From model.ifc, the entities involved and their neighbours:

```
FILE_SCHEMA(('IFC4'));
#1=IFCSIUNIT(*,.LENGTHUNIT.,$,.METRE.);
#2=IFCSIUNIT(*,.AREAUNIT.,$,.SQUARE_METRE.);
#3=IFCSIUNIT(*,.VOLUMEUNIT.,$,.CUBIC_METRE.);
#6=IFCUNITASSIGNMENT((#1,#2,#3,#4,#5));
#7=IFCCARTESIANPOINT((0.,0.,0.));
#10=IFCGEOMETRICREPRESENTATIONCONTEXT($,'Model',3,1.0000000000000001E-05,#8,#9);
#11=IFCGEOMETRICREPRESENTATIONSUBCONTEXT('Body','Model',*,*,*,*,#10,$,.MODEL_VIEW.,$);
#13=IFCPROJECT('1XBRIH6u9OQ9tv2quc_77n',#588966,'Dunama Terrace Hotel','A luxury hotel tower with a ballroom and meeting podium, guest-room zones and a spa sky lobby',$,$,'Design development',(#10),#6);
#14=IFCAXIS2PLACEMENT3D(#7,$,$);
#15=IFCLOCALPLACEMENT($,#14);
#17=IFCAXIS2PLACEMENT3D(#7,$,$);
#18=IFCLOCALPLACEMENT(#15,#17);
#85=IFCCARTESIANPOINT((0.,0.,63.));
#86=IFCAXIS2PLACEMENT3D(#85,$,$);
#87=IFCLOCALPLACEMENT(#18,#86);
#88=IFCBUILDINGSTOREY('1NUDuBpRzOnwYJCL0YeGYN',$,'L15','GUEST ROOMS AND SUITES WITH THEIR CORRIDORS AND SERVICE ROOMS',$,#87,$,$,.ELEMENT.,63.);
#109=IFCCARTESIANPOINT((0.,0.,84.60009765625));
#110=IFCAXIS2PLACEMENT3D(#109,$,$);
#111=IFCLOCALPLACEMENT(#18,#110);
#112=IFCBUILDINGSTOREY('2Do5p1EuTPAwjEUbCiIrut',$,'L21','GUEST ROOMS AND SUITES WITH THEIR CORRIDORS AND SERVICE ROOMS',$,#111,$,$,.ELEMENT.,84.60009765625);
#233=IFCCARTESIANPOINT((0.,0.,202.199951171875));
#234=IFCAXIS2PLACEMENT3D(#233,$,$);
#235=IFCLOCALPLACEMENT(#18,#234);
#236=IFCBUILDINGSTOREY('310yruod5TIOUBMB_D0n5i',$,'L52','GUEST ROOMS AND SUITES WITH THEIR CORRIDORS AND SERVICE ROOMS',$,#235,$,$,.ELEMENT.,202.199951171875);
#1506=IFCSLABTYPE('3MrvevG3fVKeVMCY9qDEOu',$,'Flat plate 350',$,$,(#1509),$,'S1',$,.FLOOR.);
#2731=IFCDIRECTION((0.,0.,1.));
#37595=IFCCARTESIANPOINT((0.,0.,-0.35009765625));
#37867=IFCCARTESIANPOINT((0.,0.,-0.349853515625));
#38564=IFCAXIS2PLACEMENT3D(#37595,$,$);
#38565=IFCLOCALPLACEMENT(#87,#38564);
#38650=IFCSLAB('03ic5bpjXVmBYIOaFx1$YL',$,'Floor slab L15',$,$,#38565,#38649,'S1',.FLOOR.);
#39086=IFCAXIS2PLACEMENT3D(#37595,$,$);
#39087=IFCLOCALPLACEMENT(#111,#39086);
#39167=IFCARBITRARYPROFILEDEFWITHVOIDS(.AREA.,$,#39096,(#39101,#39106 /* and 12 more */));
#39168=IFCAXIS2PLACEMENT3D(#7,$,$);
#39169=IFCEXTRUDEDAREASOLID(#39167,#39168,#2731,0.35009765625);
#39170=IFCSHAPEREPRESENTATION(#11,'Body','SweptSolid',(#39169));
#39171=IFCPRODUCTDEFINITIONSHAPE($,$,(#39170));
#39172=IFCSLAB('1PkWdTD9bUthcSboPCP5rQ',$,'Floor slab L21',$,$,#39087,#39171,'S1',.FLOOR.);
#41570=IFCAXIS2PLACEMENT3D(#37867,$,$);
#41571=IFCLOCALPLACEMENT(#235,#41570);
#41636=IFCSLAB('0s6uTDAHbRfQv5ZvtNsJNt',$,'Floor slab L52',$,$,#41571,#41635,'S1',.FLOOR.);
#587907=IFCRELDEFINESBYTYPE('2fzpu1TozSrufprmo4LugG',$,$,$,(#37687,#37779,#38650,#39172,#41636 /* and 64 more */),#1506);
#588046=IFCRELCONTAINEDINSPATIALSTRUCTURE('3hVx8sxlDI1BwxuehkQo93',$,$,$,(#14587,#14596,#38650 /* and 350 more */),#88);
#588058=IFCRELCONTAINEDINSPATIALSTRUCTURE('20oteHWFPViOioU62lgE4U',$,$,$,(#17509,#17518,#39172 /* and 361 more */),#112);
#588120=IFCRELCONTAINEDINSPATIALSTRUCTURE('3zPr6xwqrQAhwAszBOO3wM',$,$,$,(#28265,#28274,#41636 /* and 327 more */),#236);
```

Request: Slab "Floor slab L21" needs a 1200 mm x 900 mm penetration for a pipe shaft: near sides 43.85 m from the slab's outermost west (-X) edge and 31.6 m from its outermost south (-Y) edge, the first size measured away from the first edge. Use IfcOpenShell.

```python
import numpy as np
import ifcopenshell
import ifcopenshell.api.feature
import ifcopenshell.api.geometry
import ifcopenshell.api.root
import ifcopenshell.geom
import ifcopenshell.util.placement
import ifcopenshell.util.representation
import ifcopenshell.util.shape
import ifcopenshell.util.unit

model = ifcopenshell.open("model.ifc")
unit_scale = ifcopenshell.util.unit.calculate_unit_scale(model)
settings = ifcopenshell.geom.settings()


def volume(element):
    """Net volume in cubic metres, openings subtracted."""
    shape = ifcopenshell.geom.create_shape(settings, element)
    return ifcopenshell.util.shape.get_volume(shape.geometry)


slab = model.by_id(39172)
before = volume(slab)

# Extent in the slab's own axes, in metres. The edges named are its -X and -Y sides.
slab_shape = ifcopenshell.geom.create_shape(settings, slab)
vertices = ifcopenshell.util.shape.get_vertices(slab_shape.geometry)
x_min, y_min, bottom = vertices.min(axis=0)
top = vertices[:, 2].max()

opening = ifcopenshell.api.root.create_entity(model, ifc_class="IfcOpeningElement", name="Pipe shaft opening", predefined_type="OPENING")
context = ifcopenshell.util.representation.get_context(model, "Model", "Body", "MODEL_VIEW")
width, depth = 1.2, 0.9
outline = [(0.0, 0.0), (width, 0.0), (width, depth), (0.0, depth), (0.0, 0.0)]
# Overshoot both faces by 50 mm so the cut is clean.
shape = ifcopenshell.api.geometry.add_slab_representation(
    model, context=context, depth=top - bottom + 0.1, polyline=outline
)
ifcopenshell.api.geometry.assign_representation(model, product=opening, representation=shape)

matrix = ifcopenshell.util.placement.get_local_placement(slab.ObjectPlacement)
matrix[:, 3] = matrix @ np.append(np.array([x_min + 43.85, y_min + 31.6, bottom - 0.05]) / unit_scale, 1.0)
ifcopenshell.api.geometry.edit_object_placement(model, product=opening, matrix=matrix, is_si=False)
ifcopenshell.api.feature.add_feature(model, feature=opening, element=slab)

after = volume(slab)

print(f"slab volume {before:.3f} -> {after:.3f} m3")

model.write("model_rev.ifc")
```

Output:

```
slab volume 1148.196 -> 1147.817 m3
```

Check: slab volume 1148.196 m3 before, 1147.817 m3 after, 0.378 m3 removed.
